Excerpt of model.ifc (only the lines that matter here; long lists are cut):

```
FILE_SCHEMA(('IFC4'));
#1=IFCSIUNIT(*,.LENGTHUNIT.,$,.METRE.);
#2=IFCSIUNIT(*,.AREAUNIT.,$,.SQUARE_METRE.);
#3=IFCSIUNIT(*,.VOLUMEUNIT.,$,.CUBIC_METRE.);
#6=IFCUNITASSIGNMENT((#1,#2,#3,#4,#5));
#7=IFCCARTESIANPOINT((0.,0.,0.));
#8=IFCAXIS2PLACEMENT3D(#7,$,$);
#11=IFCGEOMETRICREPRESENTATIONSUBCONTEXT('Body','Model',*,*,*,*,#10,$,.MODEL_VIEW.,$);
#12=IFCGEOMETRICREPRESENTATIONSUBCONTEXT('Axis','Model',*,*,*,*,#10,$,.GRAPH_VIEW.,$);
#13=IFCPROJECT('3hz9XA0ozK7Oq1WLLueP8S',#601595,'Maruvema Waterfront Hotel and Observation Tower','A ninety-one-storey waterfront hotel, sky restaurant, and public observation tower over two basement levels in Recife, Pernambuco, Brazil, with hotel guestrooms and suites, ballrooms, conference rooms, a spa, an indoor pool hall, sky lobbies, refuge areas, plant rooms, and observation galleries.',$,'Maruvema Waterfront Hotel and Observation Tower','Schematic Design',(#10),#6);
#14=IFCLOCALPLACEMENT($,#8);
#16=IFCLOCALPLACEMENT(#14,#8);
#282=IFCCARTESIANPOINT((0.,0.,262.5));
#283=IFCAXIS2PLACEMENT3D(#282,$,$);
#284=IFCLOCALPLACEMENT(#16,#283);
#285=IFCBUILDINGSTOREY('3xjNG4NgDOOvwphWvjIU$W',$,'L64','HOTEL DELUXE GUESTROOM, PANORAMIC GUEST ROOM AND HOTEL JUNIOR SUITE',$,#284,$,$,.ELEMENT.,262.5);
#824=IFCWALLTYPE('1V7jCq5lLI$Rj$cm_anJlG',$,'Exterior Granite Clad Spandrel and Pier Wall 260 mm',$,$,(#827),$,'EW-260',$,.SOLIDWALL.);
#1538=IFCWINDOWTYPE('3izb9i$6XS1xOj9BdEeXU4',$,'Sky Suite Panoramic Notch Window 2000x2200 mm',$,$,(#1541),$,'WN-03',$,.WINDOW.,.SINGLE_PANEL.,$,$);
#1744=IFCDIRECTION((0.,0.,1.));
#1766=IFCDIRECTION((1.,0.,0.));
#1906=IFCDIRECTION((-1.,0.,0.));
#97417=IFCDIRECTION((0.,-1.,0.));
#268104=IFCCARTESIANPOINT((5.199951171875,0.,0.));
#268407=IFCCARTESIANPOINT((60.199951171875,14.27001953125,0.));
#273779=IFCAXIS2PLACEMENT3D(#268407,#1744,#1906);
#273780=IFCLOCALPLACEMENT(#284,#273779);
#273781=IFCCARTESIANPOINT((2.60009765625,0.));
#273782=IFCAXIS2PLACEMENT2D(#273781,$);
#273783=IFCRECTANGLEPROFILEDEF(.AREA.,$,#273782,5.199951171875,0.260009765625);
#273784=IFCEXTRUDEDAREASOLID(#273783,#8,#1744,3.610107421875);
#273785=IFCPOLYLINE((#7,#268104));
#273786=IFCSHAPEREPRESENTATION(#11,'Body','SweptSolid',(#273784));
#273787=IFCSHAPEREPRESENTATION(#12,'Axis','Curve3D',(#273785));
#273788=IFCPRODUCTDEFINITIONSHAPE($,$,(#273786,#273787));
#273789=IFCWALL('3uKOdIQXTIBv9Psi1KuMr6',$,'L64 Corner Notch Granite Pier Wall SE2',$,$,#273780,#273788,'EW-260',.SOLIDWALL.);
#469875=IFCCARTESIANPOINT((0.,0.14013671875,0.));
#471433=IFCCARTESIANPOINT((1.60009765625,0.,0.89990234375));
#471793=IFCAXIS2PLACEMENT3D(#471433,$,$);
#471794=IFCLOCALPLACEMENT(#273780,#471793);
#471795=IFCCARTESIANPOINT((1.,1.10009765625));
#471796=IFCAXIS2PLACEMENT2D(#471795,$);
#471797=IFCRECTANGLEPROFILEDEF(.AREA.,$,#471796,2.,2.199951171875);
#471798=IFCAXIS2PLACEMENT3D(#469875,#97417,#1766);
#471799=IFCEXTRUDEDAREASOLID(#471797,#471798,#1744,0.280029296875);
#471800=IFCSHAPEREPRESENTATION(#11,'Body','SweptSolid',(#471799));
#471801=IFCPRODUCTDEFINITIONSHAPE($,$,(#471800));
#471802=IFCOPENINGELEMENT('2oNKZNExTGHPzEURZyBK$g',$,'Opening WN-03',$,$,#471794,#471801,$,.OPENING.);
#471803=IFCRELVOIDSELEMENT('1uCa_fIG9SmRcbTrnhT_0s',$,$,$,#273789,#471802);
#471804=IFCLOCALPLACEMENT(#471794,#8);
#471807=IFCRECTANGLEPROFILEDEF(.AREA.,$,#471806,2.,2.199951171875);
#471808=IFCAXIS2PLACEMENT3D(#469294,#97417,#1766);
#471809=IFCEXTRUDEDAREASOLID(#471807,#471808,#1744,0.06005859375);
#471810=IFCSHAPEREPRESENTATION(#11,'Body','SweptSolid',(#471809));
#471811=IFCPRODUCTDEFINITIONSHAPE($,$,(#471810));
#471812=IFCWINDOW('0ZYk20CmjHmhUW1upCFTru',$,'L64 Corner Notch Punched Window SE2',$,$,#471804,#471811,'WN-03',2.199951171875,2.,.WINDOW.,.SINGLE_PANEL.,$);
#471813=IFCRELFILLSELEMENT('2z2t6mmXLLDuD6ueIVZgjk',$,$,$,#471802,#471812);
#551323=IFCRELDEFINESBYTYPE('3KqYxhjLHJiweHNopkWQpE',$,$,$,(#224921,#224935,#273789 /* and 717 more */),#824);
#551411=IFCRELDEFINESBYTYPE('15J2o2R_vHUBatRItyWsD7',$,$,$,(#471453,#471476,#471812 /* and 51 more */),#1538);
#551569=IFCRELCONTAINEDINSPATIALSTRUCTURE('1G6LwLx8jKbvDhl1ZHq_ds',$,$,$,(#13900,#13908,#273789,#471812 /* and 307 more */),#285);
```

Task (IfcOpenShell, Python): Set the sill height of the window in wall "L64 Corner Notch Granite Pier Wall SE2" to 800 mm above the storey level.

```python
import numpy as np
import ifcopenshell
import ifcopenshell.api.geometry
import ifcopenshell.geom
import ifcopenshell.util.element
import ifcopenshell.util.placement
import ifcopenshell.util.shape
import ifcopenshell.util.unit

model = ifcopenshell.open("model.ifc")
unit_scale = ifcopenshell.util.unit.calculate_unit_scale(model)

window = model.by_guid("0ZYk20CmjHmhUW1upCFTru")
opening = window.FillsVoids[0].RelatingOpeningElement
storey = ifcopenshell.util.element.get_container(window, ifc_class="IfcBuildingStorey")
level = ifcopenshell.util.placement.get_local_placement(storey.ObjectPlacement)[2, 3]

# The opening's origin need not be at the sill, so measure its lowest point.
shape = ifcopenshell.geom.create_shape(ifcopenshell.geom.settings(), opening)
bottom = ifcopenshell.util.shape.get_shape_bottom_elevation(shape, shape.geometry) / unit_scale
dz = level + 0.8 / unit_scale - bottom

shift = np.array([0.0, 0.0, dz])
# The window is placed relative to its opening, so it follows when the opening moves.
matrix = ifcopenshell.util.placement.get_local_placement(opening.ObjectPlacement)
matrix[:3, 3] += shift
ifcopenshell.api.geometry.edit_object_placement(
    model, product=opening, matrix=matrix, is_si=False, should_transform_children=True
)

print(f"moved by {dz * unit_scale:+.3f} m")

model.write("model_edited.ifc")
```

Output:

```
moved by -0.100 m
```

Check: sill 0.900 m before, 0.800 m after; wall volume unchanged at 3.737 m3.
